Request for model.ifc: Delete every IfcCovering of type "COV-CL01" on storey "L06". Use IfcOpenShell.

First a look at what the model holds.

```python
import ifcopenshell
import ifcopenshell.util.element

model = ifcopenshell.open("model.ifc")
print(model.schema)
storey = next(s for s in model.by_type("IfcBuildingStorey") if s.Name == "L06")
coverings = [e for e in ifcopenshell.util.element.get_decomposition(storey) if e.is_a("IfcCovering")]
seen = {}
for e in coverings:
    element_type = ifcopenshell.util.element.get_type(e)
    name = element_type.Name if element_type not in (None, e) else None
    seen[name] = seen.get(name, 0) + 1
for name, count in sorted(seen.items(), key=str):
    print(count, "x", name)
```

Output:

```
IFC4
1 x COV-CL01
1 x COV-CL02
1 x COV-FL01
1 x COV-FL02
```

```python
import ifcopenshell
import ifcopenshell.api.root
import ifcopenshell.util.element

model = ifcopenshell.open("model.ifc")

storey = next(s for s in model.by_type("IfcBuildingStorey") if s.Name == "L06")
coverings = [e for e in ifcopenshell.util.element.get_decomposition(storey) if e.is_a("IfcCovering")]
targets = [e for e in coverings if (t := ifcopenshell.util.element.get_type(e)) not in (None, e) and t.Name == "COV-CL01"]

for e in targets:
    ifcopenshell.api.root.remove_product(model, product=e)
print(len(targets), "removed")

model.write("model_edited.ifc")
```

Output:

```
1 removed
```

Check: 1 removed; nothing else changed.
